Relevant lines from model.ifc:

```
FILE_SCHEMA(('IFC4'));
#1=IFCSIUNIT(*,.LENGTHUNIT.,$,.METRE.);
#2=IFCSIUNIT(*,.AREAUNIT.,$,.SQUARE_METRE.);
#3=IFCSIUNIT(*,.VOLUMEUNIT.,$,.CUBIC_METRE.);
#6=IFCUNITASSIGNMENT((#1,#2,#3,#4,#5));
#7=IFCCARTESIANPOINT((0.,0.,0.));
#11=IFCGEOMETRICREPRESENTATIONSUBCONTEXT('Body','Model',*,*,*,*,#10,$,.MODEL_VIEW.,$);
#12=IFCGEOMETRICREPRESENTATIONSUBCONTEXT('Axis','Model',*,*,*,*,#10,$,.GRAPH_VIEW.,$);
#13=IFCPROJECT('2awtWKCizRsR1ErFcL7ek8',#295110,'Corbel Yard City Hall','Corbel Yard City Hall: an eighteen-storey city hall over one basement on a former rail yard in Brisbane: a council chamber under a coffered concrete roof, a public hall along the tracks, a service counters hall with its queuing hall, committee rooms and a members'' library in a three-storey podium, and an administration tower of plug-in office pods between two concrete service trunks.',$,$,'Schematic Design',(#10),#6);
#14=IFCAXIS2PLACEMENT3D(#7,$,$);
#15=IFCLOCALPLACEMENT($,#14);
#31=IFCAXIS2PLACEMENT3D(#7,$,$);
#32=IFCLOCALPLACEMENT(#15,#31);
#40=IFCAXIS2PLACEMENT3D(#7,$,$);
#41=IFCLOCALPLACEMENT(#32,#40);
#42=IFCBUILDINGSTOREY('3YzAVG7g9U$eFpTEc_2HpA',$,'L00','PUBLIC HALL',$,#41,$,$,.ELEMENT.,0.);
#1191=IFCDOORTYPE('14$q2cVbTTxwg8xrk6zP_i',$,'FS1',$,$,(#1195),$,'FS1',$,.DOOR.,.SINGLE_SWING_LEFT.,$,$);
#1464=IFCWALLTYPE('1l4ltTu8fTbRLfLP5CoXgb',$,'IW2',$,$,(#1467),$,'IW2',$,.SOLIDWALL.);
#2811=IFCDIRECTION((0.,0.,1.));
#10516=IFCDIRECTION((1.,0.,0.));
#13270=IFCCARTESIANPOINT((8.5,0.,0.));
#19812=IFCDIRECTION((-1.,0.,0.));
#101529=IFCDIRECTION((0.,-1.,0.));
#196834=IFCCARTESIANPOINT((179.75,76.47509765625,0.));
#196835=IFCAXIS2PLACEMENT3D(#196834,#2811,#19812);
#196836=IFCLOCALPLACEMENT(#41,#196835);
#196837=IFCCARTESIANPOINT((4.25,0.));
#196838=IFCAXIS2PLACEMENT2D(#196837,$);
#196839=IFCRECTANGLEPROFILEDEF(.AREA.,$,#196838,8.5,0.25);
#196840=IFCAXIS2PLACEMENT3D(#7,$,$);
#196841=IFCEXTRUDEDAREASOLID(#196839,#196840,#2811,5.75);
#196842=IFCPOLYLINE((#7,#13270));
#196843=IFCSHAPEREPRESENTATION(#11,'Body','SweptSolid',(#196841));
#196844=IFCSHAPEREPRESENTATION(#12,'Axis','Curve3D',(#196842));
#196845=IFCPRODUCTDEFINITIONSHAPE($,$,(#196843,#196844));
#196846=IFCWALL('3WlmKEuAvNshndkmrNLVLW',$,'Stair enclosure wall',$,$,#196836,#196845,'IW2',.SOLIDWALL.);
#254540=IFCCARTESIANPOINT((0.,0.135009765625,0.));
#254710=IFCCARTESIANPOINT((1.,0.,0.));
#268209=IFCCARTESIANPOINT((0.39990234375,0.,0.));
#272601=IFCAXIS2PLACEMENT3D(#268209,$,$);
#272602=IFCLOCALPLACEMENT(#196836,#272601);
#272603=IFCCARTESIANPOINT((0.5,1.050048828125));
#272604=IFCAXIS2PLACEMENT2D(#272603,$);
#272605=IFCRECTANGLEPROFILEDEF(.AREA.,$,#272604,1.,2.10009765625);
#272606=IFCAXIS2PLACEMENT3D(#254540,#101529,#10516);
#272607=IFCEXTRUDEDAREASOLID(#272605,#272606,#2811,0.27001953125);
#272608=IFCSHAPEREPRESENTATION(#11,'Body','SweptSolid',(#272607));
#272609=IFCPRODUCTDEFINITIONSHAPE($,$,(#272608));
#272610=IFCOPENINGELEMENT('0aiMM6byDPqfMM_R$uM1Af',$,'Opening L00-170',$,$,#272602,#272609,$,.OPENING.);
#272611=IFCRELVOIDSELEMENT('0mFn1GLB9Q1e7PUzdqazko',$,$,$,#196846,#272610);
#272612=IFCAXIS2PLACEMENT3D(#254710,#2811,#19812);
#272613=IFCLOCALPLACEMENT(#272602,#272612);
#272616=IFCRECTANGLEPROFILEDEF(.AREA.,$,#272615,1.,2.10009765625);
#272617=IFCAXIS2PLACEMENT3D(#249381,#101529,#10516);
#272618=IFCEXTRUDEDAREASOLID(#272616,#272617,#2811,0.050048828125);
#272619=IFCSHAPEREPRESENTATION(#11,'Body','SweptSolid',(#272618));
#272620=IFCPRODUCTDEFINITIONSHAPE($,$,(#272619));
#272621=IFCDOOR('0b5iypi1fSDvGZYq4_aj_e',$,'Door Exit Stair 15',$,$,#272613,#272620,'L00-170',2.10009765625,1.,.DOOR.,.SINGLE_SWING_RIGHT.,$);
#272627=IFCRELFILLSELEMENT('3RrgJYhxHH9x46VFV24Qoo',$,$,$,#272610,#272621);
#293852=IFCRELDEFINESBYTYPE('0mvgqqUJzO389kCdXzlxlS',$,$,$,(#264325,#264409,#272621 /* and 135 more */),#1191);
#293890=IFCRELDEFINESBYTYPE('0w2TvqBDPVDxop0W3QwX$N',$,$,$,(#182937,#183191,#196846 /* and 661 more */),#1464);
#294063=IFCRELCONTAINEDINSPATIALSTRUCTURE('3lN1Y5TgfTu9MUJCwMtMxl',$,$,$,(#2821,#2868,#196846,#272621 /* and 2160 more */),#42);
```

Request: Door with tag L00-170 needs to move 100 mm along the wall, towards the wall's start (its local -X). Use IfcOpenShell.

```python
import ifcopenshell
import ifcopenshell.api.geometry
import ifcopenshell.util.placement
import ifcopenshell.util.unit

model = ifcopenshell.open("model.ifc")
unit_scale = ifcopenshell.util.unit.calculate_unit_scale(model)

door = model.by_guid("0b5iypi1fSDvGZYq4_aj_e")
opening = door.FillsVoids[0].RelatingOpeningElement
wall = opening.VoidsElements[0].RelatingBuildingElement

wall_matrix = ifcopenshell.util.placement.get_local_placement(wall.ObjectPlacement)
shift = wall_matrix[:3, 0] * -0.1 / unit_scale
before = ifcopenshell.util.placement.get_local_placement(door.ObjectPlacement)[:3, 3].copy()

# The door is placed relative to its opening, so it follows when the opening moves.
matrix = ifcopenshell.util.placement.get_local_placement(opening.ObjectPlacement)
matrix[:3, 3] += shift
ifcopenshell.api.geometry.edit_object_placement(
    model, product=opening, matrix=matrix, is_si=False, should_transform_children=True
)

after = ifcopenshell.util.placement.get_local_placement(door.ObjectPlacement)[:3, 3]
print("door moved by", (after - before).round(3) + 0.0)

model.write("model_edited.ifc")
```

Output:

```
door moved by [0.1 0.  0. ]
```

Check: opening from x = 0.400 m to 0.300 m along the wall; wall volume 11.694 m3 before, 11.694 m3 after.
